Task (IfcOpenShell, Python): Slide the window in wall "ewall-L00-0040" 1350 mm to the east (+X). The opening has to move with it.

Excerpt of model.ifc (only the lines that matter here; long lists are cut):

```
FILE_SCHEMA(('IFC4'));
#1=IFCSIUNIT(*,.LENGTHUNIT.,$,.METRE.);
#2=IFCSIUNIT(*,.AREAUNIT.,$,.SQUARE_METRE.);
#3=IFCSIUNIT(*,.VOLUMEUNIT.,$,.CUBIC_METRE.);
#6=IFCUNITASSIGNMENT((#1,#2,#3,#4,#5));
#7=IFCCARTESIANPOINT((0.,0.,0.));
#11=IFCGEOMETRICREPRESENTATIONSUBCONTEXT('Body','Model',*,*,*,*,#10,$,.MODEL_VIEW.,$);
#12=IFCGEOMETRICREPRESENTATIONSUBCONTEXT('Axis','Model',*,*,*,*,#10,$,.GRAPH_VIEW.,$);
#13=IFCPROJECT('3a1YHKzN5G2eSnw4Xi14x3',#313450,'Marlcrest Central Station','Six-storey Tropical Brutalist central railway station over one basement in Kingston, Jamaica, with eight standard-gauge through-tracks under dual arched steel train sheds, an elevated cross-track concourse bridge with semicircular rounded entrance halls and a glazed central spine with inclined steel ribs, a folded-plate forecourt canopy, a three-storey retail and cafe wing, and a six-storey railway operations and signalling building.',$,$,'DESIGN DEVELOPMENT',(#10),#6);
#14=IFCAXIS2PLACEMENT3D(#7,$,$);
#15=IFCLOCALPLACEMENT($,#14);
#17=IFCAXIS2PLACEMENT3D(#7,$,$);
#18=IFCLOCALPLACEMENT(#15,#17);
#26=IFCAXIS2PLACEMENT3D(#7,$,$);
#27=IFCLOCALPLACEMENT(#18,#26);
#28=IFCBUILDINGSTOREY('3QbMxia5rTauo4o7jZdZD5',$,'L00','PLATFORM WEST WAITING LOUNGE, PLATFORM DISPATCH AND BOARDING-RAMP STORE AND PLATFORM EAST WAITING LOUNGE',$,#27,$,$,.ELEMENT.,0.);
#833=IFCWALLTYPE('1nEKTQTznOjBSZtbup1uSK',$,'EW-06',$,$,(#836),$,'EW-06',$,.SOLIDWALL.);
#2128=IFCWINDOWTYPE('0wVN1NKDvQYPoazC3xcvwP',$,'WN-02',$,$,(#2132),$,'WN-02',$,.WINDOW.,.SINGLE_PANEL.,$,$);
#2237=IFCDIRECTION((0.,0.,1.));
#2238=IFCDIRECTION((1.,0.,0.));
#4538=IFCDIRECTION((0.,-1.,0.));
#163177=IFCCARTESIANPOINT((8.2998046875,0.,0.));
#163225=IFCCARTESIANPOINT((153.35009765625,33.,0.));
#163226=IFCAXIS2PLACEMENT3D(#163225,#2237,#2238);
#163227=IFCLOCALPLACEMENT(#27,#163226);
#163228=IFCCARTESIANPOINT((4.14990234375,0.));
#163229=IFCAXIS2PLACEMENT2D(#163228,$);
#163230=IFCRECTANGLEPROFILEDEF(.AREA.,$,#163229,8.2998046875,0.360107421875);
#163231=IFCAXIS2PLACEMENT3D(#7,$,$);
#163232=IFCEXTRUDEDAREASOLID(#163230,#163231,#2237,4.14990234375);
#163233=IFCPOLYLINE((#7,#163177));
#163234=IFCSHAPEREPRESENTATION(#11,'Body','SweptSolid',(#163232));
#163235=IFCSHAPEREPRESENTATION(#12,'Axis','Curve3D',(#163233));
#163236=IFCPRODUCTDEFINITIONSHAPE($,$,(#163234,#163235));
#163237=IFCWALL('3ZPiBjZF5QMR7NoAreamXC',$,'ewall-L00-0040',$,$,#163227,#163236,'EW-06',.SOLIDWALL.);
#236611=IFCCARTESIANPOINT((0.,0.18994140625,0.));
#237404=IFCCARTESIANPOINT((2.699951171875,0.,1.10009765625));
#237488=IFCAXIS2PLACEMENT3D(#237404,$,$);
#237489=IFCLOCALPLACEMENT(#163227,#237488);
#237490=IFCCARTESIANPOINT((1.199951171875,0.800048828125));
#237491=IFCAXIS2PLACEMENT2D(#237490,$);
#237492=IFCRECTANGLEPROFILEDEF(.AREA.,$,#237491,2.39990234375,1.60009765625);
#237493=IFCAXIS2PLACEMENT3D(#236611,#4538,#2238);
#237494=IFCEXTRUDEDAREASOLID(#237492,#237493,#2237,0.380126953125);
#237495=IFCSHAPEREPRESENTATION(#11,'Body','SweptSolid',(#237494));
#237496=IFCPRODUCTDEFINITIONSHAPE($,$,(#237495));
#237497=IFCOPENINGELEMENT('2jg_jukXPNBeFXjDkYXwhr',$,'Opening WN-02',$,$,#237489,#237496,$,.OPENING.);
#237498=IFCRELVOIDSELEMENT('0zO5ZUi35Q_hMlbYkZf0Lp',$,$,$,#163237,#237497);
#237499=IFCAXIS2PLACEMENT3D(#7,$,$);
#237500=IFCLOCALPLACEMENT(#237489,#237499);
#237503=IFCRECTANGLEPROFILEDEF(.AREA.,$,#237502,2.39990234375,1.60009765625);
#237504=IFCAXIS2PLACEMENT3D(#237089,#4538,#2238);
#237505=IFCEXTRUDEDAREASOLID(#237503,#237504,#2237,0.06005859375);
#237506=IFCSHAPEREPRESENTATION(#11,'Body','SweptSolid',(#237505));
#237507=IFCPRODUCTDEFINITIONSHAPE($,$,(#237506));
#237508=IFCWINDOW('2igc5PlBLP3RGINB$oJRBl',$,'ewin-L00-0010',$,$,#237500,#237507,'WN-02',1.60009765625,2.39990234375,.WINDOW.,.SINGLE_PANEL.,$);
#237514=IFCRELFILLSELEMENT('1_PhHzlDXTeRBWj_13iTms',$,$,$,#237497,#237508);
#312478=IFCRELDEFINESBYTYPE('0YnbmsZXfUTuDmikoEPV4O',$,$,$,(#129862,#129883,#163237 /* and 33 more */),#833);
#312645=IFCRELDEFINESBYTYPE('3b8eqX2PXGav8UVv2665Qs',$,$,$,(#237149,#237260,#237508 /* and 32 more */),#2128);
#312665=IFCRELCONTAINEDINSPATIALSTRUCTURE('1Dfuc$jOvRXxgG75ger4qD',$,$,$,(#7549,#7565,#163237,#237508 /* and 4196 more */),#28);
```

```python
import ifcopenshell
import ifcopenshell.api.geometry
import ifcopenshell.util.placement
import ifcopenshell.util.unit

model = ifcopenshell.open("model.ifc")
unit_scale = ifcopenshell.util.unit.calculate_unit_scale(model)

window = model.by_guid("2igc5PlBLP3RGINB$oJRBl")
opening = window.FillsVoids[0].RelatingOpeningElement
wall = opening.VoidsElements[0].RelatingBuildingElement

wall_matrix = ifcopenshell.util.placement.get_local_placement(wall.ObjectPlacement)
shift = wall_matrix[:3, 0] * 1.35 / unit_scale
before = ifcopenshell.util.placement.get_local_placement(window.ObjectPlacement)[:3, 3].copy()

# The window is placed relative to its opening, so it follows when the opening moves.
matrix = ifcopenshell.util.placement.get_local_placement(opening.ObjectPlacement)
matrix[:3, 3] += shift
ifcopenshell.api.geometry.edit_object_placement(
    model, product=opening, matrix=matrix, is_si=False, should_transform_children=True
)

after = ifcopenshell.util.placement.get_local_placement(window.ObjectPlacement)[:3, 3]
print("window moved by", (after - before).round(3) + 0.0)

model.write("model-out.ifc")
```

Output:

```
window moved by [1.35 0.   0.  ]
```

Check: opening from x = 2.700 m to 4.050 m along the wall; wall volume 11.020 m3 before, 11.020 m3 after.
